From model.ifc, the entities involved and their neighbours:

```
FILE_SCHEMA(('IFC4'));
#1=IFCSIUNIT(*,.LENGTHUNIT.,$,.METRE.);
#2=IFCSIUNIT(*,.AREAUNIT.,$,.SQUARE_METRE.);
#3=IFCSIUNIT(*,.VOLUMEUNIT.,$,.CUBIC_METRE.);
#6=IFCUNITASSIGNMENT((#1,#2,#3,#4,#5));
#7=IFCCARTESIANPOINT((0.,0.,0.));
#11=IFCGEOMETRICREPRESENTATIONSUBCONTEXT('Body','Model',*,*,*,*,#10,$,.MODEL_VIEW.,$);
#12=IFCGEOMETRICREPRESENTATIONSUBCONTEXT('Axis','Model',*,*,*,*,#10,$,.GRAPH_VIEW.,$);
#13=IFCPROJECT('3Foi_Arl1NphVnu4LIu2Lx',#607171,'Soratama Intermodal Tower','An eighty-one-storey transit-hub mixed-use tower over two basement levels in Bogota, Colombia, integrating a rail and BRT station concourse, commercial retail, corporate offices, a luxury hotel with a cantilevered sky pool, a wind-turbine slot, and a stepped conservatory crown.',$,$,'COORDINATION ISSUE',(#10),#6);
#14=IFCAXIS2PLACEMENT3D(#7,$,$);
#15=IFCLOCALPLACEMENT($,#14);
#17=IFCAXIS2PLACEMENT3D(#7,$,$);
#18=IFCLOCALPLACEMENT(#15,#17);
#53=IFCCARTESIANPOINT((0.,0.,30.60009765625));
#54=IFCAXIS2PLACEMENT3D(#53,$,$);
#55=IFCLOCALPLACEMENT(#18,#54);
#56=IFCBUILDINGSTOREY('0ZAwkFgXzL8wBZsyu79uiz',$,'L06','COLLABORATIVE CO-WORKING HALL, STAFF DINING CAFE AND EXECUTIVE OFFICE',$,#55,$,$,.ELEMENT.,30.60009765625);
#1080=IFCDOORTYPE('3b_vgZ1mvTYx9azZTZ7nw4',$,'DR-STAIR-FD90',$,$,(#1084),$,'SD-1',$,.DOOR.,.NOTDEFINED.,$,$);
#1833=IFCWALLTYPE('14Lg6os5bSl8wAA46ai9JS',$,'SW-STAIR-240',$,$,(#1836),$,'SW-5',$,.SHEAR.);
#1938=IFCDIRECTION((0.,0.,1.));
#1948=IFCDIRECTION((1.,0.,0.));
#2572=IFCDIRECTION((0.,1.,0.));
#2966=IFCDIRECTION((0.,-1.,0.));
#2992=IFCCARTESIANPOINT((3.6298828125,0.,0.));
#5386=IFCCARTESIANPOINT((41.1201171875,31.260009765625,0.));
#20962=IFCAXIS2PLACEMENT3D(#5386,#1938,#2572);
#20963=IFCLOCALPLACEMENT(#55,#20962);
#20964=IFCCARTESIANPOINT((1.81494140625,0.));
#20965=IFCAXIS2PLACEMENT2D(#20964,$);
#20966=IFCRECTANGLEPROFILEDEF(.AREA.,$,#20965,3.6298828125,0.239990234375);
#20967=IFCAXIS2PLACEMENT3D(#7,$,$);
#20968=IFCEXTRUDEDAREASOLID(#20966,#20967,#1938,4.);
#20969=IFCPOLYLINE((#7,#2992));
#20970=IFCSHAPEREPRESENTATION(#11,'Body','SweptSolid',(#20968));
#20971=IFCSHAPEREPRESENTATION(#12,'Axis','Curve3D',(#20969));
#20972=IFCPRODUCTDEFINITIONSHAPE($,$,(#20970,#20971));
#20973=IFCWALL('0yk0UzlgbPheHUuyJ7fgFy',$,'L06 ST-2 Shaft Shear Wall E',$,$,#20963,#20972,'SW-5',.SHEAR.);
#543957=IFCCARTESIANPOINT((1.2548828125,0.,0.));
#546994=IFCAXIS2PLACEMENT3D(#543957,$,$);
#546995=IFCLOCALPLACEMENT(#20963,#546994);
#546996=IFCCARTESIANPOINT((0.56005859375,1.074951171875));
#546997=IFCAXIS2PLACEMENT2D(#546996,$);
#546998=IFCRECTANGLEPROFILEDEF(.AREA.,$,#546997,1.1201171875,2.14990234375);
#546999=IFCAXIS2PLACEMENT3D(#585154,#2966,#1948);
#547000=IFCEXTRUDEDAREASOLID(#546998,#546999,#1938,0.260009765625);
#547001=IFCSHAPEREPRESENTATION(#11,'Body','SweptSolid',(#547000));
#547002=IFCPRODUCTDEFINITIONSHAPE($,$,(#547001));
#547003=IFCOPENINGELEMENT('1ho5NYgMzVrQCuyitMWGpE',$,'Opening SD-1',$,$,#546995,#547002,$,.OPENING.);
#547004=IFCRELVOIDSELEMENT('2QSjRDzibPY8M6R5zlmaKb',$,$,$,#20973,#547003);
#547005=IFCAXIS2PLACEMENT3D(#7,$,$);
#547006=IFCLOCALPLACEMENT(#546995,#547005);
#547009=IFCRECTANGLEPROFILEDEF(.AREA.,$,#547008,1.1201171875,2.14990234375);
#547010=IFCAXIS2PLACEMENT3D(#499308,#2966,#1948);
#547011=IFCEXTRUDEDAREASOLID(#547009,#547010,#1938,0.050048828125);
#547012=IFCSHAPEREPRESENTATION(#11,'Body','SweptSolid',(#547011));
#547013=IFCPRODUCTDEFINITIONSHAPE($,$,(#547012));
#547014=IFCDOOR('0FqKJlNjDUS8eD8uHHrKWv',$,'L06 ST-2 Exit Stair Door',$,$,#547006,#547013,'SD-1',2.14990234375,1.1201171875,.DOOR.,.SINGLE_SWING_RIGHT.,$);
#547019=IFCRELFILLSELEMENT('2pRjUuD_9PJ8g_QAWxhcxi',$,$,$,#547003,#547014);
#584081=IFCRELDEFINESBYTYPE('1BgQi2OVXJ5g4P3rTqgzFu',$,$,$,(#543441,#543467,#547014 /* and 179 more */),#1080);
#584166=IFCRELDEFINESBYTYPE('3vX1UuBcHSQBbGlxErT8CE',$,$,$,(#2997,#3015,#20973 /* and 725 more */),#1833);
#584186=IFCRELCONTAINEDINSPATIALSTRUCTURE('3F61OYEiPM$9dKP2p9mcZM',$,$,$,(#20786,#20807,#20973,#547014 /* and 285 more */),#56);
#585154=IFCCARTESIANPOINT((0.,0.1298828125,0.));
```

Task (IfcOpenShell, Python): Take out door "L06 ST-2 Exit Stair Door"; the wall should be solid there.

```python
import ifcopenshell
import ifcopenshell.api.feature
import ifcopenshell.api.root
import ifcopenshell.geom
import ifcopenshell.util.shape

model = ifcopenshell.open("model.ifc")
settings = ifcopenshell.geom.settings()


def volume(element):
    """Net volume in cubic metres, openings subtracted."""
    shape = ifcopenshell.geom.create_shape(settings, element)
    return ifcopenshell.util.shape.get_volume(shape.geometry)


door = model.by_guid("0FqKJlNjDUS8eD8uHHrKWv")
opening = door.FillsVoids[0].RelatingOpeningElement
wall = opening.VoidsElements[0].RelatingBuildingElement
before = volume(wall)

ifcopenshell.api.root.remove_product(model, product=door)
ifcopenshell.api.feature.remove_feature(model, feature=opening)

after = volume(wall)

print(f"wall volume {before:.3f} -> {after:.3f} m3")

model.write("model_rev.ifc")
```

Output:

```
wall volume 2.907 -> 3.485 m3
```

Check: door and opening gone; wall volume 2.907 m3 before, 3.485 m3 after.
